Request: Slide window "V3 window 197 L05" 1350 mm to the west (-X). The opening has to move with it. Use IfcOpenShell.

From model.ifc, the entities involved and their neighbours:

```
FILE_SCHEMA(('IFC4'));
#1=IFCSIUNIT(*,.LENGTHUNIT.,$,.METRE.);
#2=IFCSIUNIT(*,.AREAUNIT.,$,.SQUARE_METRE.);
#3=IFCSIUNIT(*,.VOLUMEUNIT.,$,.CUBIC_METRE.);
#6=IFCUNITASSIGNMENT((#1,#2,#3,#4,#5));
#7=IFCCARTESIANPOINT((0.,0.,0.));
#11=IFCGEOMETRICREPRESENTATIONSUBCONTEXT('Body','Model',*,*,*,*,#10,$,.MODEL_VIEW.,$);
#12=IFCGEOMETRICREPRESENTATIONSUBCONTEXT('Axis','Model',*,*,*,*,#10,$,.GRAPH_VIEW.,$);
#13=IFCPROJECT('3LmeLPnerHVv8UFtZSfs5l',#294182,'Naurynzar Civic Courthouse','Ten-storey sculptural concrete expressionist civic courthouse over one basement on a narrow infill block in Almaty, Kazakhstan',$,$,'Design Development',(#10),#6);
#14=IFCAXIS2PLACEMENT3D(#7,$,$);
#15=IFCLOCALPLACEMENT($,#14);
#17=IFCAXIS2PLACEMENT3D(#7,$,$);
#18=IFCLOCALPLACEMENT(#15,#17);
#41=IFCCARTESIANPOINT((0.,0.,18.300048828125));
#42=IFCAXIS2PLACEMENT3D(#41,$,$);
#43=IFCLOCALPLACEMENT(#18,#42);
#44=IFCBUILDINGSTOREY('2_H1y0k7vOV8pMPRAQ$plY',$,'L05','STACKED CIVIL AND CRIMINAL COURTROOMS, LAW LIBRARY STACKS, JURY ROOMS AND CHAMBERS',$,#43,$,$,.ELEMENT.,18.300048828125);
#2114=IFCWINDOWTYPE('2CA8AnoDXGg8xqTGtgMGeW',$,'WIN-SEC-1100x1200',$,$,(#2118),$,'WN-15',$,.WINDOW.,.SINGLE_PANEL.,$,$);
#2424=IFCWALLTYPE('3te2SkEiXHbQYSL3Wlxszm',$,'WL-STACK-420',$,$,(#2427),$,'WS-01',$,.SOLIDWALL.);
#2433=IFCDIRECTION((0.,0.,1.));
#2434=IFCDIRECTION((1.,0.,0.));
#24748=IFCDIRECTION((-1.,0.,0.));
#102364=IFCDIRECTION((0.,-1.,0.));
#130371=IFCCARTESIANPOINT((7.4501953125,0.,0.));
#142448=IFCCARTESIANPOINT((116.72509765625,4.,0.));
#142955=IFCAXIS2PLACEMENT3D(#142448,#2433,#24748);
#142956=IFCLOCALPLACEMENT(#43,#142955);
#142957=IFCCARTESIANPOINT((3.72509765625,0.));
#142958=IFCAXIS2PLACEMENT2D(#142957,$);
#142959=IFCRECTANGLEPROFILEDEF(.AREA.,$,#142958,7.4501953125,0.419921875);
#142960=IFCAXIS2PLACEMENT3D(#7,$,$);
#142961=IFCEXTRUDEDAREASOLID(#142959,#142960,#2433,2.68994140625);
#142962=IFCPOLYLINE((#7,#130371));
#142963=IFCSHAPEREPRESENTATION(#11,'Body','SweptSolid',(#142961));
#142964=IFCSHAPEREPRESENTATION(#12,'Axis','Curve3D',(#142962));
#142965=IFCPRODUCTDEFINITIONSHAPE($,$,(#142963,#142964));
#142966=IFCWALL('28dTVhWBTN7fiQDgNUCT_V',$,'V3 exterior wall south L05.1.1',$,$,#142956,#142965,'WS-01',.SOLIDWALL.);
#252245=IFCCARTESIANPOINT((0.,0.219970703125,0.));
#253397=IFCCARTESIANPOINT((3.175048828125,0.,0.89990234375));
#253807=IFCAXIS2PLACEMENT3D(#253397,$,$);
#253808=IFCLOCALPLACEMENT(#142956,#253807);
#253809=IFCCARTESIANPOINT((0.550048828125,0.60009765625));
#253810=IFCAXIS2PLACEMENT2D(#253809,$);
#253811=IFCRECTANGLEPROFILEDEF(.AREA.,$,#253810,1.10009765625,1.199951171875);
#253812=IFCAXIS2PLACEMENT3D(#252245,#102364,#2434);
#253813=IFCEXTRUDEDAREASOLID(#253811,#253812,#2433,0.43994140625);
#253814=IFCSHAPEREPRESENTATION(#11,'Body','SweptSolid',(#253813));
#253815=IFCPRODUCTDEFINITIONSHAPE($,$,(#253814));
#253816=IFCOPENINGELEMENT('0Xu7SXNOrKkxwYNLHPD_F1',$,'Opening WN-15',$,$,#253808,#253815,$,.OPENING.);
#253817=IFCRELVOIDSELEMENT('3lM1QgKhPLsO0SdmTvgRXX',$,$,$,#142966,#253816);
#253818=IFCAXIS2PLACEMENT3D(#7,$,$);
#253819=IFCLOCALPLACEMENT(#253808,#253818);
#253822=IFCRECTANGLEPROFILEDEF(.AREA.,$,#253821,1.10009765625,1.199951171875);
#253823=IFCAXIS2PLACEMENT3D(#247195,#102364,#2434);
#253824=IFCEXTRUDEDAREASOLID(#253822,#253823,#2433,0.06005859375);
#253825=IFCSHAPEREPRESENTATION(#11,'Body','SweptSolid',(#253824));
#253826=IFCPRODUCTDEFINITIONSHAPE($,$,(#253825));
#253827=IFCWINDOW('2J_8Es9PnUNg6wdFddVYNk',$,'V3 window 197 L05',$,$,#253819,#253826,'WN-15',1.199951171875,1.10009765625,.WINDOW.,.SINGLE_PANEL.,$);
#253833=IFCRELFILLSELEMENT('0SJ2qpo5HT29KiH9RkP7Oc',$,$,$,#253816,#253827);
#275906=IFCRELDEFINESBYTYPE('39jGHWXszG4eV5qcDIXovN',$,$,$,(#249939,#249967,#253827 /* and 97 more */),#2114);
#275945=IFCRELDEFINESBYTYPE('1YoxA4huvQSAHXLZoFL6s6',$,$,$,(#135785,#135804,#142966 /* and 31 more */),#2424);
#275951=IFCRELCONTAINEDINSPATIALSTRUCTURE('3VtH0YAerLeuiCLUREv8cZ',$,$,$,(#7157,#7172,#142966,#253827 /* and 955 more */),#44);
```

```python
import ifcopenshell
import ifcopenshell.api.geometry
import ifcopenshell.util.placement
import ifcopenshell.util.unit

model = ifcopenshell.open("model.ifc")
unit_scale = ifcopenshell.util.unit.calculate_unit_scale(model)

window = model.by_id(253827)
opening = window.FillsVoids[0].RelatingOpeningElement
wall = opening.VoidsElements[0].RelatingBuildingElement

wall_matrix = ifcopenshell.util.placement.get_local_placement(wall.ObjectPlacement)
shift = wall_matrix[:3, 0] * 1.35 / unit_scale
before = ifcopenshell.util.placement.get_local_placement(window.ObjectPlacement)[:3, 3].copy()

# The window is placed relative to its opening, so it follows when the opening moves.
matrix = ifcopenshell.util.placement.get_local_placement(opening.ObjectPlacement)
matrix[:3, 3] += shift
ifcopenshell.api.geometry.edit_object_placement(
    model, product=opening, matrix=matrix, is_si=False, should_transform_children=True
)

after = ifcopenshell.util.placement.get_local_placement(window.ObjectPlacement)[:3, 3]
print("window moved by", (after - before).round(3) + 0.0)

model.write("model-out.ifc")
```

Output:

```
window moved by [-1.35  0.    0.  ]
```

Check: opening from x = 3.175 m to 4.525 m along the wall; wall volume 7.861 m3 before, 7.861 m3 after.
